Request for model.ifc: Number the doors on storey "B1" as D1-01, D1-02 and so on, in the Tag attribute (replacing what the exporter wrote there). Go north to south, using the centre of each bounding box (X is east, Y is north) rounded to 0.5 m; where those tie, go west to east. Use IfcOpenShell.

First a look at what the model holds.

```python
import ifcopenshell
import ifcopenshell.util.element
import ifcopenshell.util.placement

model = ifcopenshell.open("model.ifc")
print(model.schema)
storey = next(s for s in model.by_type("IfcBuildingStorey") if s.Name == "B1")
doors = [e for e in ifcopenshell.util.element.get_decomposition(storey) if e.is_a("IfcDoor")]
for e in sorted(doors, key=lambda e: e.id()):
    origin = ifcopenshell.util.placement.get_local_placement(e.ObjectPlacement)[:3, 3]
    print(e.id(), e.Tag, e.Name, origin.round(2) + 0.0, sep=" | ")
```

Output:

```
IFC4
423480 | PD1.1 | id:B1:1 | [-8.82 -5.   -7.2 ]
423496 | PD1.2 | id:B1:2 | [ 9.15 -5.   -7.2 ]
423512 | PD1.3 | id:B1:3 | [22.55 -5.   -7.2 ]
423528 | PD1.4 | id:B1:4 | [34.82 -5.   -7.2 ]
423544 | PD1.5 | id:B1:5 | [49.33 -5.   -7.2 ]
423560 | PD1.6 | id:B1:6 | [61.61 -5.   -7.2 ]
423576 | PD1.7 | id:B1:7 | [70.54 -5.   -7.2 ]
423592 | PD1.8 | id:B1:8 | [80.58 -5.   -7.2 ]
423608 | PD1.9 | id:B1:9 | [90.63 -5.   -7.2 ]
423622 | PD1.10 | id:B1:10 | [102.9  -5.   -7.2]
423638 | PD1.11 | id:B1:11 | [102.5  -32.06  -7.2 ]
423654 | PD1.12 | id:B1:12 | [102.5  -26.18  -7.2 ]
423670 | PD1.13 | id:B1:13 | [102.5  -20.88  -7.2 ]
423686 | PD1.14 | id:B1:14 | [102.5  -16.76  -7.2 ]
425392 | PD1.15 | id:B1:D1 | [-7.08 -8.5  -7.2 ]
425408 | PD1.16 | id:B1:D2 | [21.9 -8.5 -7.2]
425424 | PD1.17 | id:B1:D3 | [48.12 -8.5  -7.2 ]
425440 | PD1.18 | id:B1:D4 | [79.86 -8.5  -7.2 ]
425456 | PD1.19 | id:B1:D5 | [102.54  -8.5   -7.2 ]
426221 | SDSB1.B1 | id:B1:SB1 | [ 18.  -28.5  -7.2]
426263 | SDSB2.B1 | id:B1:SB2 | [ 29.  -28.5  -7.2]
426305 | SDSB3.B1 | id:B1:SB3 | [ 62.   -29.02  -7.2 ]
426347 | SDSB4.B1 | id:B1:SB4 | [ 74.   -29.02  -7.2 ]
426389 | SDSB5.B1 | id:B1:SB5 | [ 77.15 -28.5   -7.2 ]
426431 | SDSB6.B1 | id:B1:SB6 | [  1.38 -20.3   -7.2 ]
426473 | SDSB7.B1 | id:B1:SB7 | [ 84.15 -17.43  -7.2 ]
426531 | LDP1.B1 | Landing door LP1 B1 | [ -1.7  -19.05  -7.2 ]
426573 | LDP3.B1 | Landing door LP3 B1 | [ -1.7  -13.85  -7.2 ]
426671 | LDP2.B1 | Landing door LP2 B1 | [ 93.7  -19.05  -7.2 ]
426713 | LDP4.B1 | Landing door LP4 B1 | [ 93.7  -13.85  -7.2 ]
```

```python
import ifcopenshell
import ifcopenshell.geom
import ifcopenshell.util.element
import ifcopenshell.util.shape

model = ifcopenshell.open("model.ifc")
settings = ifcopenshell.geom.settings()
settings.set("use-world-coords", True)


def centre(element):
    shape = ifcopenshell.geom.create_shape(settings, element)
    return ifcopenshell.util.shape.get_bbox_centroid(shape.geometry)


storey = next(s for s in model.by_type("IfcBuildingStorey") if s.Name == "B1")
doors = [e for e in ifcopenshell.util.element.get_decomposition(storey) if e.is_a("IfcDoor")]

# Insertion points can sit at a corner or the storey origin, so sort by the geometry (in metres).
centres = {e: centre(e) for e in doors}
doors.sort(key=lambda e: (-round(centres[e][1] / 0.5), centres[e][0]))

for i, e in enumerate(doors, start=1):
    number = f"D1-{i:02d}"
    e.Tag = number
    print(e.id(), number)

model.write("model_v2.ifc")
```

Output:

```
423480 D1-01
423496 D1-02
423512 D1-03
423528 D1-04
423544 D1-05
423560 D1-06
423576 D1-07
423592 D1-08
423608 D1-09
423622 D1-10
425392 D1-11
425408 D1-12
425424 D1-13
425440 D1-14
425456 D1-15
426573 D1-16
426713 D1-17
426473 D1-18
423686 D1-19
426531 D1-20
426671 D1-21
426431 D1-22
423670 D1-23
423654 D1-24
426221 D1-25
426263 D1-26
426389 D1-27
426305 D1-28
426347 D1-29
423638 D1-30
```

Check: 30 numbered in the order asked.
